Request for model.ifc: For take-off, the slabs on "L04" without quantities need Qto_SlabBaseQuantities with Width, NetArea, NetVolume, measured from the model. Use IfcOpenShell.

First a look at what the model holds.

```python
import ifcopenshell
import ifcopenshell.util.element
import ifcopenshell.util.unit

model = ifcopenshell.open("model.ifc")
print(model.schema)
for unit_type in ("LENGTHUNIT", "AREAUNIT", "VOLUMEUNIT"):
    print(unit_type, ifcopenshell.util.unit.calculate_unit_scale(model, unit_type))
storey = next(s for s in model.by_type("IfcBuildingStorey") if s.Name == "L04")
slabs = [e for e in ifcopenshell.util.element.get_decomposition(storey) if e.is_a("IfcSlab")]
for e in sorted(slabs, key=lambda e: e.id()):
    print(e.id(), e.is_a(), e.Name, list(ifcopenshell.util.element.get_psets(e, qtos_only=True)), sep=" | ")
```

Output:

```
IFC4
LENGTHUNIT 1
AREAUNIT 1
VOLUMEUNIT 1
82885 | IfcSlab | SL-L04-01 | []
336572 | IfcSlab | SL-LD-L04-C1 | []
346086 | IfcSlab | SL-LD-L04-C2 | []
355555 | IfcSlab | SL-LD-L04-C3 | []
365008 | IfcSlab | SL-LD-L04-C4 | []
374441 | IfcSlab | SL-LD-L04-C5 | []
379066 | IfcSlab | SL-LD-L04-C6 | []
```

```python
import ifcopenshell
import ifcopenshell.api.pset
import ifcopenshell.geom
import ifcopenshell.util.element
import ifcopenshell.util.shape
import ifcopenshell.util.unit

model = ifcopenshell.open("model.ifc")
unit_scale = ifcopenshell.util.unit.calculate_unit_scale(model)
area_scale = ifcopenshell.util.unit.calculate_unit_scale(model, "AREAUNIT")
volume_scale = ifcopenshell.util.unit.calculate_unit_scale(model, "VOLUMEUNIT")
settings = ifcopenshell.geom.settings()

storey = next(s for s in model.by_type("IfcBuildingStorey") if s.Name == "L04")
slabs = [e for e in ifcopenshell.util.element.get_decomposition(storey) if e.is_a("IfcSlab")]

for e in sorted(slabs, key=lambda e: e.id()):
    if ifcopenshell.util.element.get_psets(e, qtos_only=True, should_inherit=False):
        continue
    # Geometry comes back in metres, in the element's own axes.
    shape = ifcopenshell.geom.create_shape(settings, e)
    values = {
        "Width": ifcopenshell.util.shape.get_z(shape.geometry) / unit_scale,
        "NetArea": ifcopenshell.util.shape.get_footprint_area(shape.geometry) / area_scale,
        "NetVolume": ifcopenshell.util.shape.get_volume(shape.geometry) / volume_scale,
    }
    qto = ifcopenshell.api.pset.add_qto(model, product=e, name="Qto_SlabBaseQuantities")
    ifcopenshell.api.pset.edit_qto(model, qto=qto, properties=values)
    print(e.id(), {k: round(v, 3) for k, v in values.items()})

model.write("model-out.ifc")
```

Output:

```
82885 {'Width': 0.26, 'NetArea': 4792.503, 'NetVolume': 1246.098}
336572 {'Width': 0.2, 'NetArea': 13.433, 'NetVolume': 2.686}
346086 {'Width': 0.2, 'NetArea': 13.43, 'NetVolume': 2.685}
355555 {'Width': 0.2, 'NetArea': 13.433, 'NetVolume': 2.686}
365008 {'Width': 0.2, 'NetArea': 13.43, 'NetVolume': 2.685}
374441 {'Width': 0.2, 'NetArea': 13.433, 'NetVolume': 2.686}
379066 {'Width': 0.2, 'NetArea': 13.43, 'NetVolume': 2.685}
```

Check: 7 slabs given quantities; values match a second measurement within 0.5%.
